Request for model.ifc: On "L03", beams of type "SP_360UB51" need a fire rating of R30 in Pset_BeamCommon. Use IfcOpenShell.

First a look at what the model holds.

```python
import ifcopenshell
import ifcopenshell.util.element

model = ifcopenshell.open("model.ifc")
print(model.schema)
storey = next(s for s in model.by_type("IfcBuildingStorey") if s.Name == "L03")
beams = [e for e in ifcopenshell.util.element.get_decomposition(storey) if e.is_a("IfcBeam")]
seen = {}
for e in beams:
    element_type = ifcopenshell.util.element.get_type(e)
    key = (element_type.Name if element_type != e and element_type else None, ifcopenshell.util.element.get_pset(e, "Pset_BeamCommon", "FireRating"))
    seen[key] = seen.get(key, 0) + 1
for (name, value), count in sorted(seen.items(), key=str):
    print(count, "x", name, "|", value)
```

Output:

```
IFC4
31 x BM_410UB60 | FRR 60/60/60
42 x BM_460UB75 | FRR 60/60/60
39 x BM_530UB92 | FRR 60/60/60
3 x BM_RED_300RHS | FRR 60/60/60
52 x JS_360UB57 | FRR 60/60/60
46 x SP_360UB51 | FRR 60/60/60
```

```python
import ifcopenshell
import ifcopenshell.api.pset
import ifcopenshell.util.element

model = ifcopenshell.open("model.ifc")

storey = next(s for s in model.by_type("IfcBuildingStorey") if s.Name == "L03")
beams = [e for e in ifcopenshell.util.element.get_decomposition(storey) if e.is_a("IfcBeam")]

count = 0
for e in beams:
    element_type = ifcopenshell.util.element.get_type(e)
    if element_type in (None, e) or element_type.Name != "SP_360UB51":
        continue
    # add_pset returns the element's existing set when there is one.
    pset = ifcopenshell.api.pset.add_pset(model, product=e, name="Pset_BeamCommon")
    ifcopenshell.api.pset.edit_pset(model, pset=pset, properties={"FireRating": "R30"})
    count += 1

print(count, "beams updated")

model.write("model-out.ifc")
```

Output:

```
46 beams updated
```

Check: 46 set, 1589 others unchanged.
